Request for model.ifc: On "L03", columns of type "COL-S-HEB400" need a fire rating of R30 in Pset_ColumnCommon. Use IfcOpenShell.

First a look at what the model holds.

```python
import ifcopenshell
import ifcopenshell.util.element

model = ifcopenshell.open("model.ifc")
print(model.schema)
storey = next(s for s in model.by_type("IfcBuildingStorey") if s.Name == "L03")
columns = [e for e in ifcopenshell.util.element.get_decomposition(storey) if e.is_a("IfcColumn")]
seen = {}
for e in columns:
    element_type = ifcopenshell.util.element.get_type(e)
    key = (element_type.Name if element_type != e and element_type else None, ifcopenshell.util.element.get_pset(e, "Pset_ColumnCommon", "FireRating"))
    seen[key] = seen.get(key, 0) + 1
for (name, value), count in sorted(seen.items(), key=str):
    print(count, "x", name, "|", value)
```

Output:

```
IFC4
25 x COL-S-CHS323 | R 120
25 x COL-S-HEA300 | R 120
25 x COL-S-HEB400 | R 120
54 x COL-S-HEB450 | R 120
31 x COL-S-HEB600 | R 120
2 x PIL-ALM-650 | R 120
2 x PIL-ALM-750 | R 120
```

```python
import ifcopenshell
import ifcopenshell.api.pset
import ifcopenshell.util.element

model = ifcopenshell.open("model.ifc")

storey = next(s for s in model.by_type("IfcBuildingStorey") if s.Name == "L03")
columns = [e for e in ifcopenshell.util.element.get_decomposition(storey) if e.is_a("IfcColumn")]

count = 0
for e in columns:
    element_type = ifcopenshell.util.element.get_type(e)
    if element_type in (None, e) or element_type.Name != "COL-S-HEB400":
        continue
    # add_pset returns the element's existing set when there is one.
    pset = ifcopenshell.api.pset.add_pset(model, product=e, name="Pset_ColumnCommon")
    ifcopenshell.api.pset.edit_pset(model, pset=pset, properties={"FireRating": "R30"})
    count += 1

print(count, "columns updated")

model.write("model_edited.ifc")
```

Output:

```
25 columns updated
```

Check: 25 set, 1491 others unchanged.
